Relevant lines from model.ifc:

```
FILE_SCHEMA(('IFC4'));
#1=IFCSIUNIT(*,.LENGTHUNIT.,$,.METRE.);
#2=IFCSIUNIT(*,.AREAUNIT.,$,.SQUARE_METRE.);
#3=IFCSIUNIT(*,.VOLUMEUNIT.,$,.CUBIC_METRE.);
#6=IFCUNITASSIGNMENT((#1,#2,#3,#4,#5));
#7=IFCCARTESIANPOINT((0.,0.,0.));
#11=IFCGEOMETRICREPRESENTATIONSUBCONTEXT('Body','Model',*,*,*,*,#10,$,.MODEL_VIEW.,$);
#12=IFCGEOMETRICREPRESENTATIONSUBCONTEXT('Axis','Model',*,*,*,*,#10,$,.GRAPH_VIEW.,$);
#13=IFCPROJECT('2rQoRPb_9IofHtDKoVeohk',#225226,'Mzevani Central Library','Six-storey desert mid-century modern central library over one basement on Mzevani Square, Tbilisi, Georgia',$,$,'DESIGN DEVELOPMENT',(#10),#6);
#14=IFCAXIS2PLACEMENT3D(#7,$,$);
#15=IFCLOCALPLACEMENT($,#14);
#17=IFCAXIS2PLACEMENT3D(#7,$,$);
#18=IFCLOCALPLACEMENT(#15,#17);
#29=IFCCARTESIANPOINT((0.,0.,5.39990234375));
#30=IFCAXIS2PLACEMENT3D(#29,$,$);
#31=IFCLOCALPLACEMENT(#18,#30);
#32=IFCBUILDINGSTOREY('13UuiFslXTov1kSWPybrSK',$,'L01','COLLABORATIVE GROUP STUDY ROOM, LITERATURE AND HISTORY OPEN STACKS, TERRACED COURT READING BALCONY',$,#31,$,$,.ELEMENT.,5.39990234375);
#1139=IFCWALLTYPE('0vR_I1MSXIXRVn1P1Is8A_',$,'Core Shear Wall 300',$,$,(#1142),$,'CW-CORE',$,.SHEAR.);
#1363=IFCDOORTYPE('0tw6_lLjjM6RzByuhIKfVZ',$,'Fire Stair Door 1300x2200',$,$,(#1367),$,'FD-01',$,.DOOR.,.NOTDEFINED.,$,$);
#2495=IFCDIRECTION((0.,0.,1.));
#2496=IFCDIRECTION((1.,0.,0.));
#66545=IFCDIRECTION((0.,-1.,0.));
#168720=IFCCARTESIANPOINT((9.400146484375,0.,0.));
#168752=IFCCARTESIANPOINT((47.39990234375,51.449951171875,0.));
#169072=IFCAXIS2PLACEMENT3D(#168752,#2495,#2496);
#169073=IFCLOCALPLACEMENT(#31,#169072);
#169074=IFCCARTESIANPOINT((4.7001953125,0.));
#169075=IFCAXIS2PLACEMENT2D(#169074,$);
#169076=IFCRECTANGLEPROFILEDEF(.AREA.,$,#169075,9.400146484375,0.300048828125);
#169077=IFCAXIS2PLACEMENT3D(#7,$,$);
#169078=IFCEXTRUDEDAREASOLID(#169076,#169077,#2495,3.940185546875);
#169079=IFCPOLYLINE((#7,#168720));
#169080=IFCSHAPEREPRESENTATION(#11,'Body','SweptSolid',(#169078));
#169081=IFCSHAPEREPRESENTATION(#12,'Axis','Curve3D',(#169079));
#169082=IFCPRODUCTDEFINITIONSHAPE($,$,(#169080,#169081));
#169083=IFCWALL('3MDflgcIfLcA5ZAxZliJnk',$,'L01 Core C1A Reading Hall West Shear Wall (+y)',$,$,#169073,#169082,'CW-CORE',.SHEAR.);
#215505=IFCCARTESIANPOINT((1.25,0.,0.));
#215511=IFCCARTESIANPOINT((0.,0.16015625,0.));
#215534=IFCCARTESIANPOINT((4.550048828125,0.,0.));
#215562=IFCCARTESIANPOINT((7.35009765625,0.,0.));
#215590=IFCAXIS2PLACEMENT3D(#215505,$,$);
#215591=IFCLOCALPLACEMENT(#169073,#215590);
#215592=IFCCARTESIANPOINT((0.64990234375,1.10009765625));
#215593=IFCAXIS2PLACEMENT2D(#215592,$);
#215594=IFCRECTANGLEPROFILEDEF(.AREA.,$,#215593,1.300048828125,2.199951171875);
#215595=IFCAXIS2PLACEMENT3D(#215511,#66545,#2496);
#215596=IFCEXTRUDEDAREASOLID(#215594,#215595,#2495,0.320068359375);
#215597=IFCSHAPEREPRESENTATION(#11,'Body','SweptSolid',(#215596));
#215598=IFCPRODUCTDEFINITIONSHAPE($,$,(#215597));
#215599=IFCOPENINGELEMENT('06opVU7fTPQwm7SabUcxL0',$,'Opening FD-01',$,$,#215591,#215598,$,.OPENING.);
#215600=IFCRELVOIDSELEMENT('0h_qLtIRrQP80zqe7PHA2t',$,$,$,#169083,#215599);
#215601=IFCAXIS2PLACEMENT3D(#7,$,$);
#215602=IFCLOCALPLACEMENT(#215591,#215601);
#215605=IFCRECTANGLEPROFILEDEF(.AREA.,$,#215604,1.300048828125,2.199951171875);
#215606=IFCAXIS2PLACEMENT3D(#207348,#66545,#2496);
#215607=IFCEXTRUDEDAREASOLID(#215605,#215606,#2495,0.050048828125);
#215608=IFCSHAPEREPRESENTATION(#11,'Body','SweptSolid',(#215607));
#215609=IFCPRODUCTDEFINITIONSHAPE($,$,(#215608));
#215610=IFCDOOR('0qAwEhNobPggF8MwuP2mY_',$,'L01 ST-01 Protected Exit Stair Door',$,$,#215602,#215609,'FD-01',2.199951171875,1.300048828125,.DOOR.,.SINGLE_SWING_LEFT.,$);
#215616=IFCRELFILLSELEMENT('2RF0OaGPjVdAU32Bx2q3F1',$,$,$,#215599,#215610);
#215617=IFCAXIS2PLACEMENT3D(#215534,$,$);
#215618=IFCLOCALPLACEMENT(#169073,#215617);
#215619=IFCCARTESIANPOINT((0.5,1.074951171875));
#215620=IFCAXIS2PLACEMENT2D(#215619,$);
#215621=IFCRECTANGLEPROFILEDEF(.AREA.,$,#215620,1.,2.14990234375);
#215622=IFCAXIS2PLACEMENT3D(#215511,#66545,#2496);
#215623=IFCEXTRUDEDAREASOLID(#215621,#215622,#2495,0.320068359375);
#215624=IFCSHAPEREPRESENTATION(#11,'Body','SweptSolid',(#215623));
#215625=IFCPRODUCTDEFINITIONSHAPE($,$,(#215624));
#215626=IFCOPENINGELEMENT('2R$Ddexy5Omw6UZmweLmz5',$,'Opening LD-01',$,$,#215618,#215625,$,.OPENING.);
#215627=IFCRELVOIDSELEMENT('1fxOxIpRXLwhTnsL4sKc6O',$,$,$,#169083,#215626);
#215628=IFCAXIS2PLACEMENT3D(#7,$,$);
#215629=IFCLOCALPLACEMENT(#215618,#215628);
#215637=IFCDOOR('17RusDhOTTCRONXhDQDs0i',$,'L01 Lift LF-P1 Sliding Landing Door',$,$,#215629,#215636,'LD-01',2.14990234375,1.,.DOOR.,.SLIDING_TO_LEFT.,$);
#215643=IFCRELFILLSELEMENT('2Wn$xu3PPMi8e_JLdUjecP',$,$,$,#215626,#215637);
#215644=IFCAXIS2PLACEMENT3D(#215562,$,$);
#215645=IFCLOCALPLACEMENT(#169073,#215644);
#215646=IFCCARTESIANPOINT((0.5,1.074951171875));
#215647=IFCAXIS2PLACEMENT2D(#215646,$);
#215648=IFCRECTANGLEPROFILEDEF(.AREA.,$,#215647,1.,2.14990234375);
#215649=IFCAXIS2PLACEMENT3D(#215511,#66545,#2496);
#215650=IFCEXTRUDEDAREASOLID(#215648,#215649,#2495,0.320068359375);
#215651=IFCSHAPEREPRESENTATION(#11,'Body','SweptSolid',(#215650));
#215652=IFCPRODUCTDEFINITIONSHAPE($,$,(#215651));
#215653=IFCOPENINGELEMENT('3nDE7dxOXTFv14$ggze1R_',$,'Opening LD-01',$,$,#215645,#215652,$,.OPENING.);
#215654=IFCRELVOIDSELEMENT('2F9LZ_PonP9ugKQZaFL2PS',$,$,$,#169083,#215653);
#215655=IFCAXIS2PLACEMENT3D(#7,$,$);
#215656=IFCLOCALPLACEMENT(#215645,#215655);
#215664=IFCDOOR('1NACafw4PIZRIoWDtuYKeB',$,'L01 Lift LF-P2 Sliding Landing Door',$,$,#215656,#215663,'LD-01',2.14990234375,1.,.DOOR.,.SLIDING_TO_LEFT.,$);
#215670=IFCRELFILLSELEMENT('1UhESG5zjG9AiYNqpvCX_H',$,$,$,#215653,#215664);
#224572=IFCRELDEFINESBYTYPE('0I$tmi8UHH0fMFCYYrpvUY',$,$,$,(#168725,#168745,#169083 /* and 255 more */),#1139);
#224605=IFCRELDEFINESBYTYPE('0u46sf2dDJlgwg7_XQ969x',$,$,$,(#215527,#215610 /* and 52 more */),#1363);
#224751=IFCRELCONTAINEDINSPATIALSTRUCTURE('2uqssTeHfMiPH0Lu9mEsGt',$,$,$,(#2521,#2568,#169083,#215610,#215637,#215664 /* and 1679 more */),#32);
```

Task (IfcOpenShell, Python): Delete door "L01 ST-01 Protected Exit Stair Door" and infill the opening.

```python
import ifcopenshell
import ifcopenshell.api.feature
import ifcopenshell.api.root
import ifcopenshell.geom
import ifcopenshell.util.shape

model = ifcopenshell.open("model.ifc")
settings = ifcopenshell.geom.settings()


def volume(element):
    """Net volume in cubic metres, openings subtracted."""
    shape = ifcopenshell.geom.create_shape(settings, element)
    return ifcopenshell.util.shape.get_volume(shape.geometry)


door = model.by_guid("0qAwEhNobPggF8MwuP2mY_")
opening = door.FillsVoids[0].RelatingOpeningElement
wall = opening.VoidsElements[0].RelatingBuildingElement
before = volume(wall)

ifcopenshell.api.root.remove_product(model, product=door)
ifcopenshell.api.feature.remove_feature(model, feature=opening)

after = volume(wall)

print(f"wall volume {before:.3f} -> {after:.3f} m3")

model.write("model_updated.ifc")
```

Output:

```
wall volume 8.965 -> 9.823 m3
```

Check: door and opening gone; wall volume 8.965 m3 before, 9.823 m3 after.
